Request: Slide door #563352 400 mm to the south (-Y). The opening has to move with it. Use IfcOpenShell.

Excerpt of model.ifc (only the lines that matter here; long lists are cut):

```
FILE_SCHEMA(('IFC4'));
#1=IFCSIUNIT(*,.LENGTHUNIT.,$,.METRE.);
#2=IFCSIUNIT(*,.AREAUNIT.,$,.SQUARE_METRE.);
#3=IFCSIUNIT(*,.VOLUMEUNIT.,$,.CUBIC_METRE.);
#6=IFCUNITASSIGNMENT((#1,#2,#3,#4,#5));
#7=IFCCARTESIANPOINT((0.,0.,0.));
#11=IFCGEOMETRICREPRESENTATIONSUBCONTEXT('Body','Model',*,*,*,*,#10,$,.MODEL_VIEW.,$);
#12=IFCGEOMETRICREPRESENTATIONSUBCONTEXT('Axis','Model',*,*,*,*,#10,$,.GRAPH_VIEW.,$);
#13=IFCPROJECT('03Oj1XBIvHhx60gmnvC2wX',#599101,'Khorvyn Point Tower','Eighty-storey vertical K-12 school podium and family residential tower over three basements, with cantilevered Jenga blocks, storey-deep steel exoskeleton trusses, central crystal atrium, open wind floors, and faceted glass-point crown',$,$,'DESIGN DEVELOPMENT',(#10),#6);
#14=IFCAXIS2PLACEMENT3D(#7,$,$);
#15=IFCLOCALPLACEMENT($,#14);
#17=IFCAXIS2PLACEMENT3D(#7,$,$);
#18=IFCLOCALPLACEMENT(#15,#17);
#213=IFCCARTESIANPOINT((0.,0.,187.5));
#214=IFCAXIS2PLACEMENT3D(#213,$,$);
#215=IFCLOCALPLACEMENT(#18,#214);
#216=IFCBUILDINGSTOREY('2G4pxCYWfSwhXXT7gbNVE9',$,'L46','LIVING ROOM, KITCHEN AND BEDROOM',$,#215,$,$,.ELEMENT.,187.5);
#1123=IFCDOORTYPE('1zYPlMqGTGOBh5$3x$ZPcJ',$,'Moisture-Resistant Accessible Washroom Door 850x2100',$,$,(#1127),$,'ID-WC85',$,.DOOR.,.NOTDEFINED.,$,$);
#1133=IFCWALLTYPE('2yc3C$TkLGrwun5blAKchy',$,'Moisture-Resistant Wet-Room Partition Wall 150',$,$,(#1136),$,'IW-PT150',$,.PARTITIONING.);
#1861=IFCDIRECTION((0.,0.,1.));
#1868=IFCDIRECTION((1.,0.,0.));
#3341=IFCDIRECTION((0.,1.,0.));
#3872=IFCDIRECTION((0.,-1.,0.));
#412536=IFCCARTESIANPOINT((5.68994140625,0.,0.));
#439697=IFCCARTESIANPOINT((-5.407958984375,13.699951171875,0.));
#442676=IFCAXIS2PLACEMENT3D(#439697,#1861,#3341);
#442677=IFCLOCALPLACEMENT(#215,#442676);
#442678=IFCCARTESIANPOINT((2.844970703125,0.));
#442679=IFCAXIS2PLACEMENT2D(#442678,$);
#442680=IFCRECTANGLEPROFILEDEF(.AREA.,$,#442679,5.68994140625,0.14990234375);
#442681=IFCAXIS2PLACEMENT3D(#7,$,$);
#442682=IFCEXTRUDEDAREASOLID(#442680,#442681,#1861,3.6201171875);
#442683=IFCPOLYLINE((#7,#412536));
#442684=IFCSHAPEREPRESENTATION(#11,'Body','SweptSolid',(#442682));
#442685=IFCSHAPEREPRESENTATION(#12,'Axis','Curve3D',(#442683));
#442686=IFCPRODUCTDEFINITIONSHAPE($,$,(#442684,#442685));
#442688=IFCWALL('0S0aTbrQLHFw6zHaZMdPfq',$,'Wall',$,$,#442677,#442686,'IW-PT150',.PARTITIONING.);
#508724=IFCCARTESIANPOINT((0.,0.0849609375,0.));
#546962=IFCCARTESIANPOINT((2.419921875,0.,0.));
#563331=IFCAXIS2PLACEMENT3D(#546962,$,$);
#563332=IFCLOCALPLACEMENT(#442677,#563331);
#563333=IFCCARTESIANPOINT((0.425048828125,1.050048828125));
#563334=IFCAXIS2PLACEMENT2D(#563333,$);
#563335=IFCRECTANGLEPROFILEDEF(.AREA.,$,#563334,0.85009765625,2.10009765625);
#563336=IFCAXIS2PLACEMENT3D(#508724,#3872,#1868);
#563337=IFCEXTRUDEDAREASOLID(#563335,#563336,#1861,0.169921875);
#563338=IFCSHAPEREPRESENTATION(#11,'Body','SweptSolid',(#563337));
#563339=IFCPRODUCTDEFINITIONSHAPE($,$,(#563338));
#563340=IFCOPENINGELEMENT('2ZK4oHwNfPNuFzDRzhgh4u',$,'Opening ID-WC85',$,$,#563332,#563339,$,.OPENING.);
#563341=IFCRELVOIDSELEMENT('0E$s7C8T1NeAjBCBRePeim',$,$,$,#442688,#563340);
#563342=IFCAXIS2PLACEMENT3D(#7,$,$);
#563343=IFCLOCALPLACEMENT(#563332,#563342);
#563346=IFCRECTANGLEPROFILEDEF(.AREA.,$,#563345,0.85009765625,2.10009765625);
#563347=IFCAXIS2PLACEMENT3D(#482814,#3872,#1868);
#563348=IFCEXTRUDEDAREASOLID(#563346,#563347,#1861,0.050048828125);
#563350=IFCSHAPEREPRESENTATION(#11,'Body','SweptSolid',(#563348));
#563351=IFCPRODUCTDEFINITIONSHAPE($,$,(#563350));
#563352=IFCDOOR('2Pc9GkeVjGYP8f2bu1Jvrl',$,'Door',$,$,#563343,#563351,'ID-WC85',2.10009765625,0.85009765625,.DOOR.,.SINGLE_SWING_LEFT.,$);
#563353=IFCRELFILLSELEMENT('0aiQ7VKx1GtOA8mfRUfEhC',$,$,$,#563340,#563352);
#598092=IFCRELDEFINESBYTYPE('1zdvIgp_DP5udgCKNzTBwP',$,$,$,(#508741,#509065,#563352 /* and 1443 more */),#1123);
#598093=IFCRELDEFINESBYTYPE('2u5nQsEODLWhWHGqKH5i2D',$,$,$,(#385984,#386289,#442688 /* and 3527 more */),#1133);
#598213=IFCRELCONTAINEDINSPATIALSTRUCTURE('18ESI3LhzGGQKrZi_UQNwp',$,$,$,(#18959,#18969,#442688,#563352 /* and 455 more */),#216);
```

```python
import ifcopenshell
import ifcopenshell.api.geometry
import ifcopenshell.util.placement

model = ifcopenshell.open("model.ifc")

door = model.by_guid("2Pc9GkeVjGYP8f2bu1Jvrl")
opening = door.FillsVoids[0].RelatingOpeningElement
wall = opening.VoidsElements[0].RelatingBuildingElement

wall_matrix = ifcopenshell.util.placement.get_local_placement(wall.ObjectPlacement)
shift = wall_matrix[:3, 0] * -0.4
before = ifcopenshell.util.placement.get_local_placement(door.ObjectPlacement)[:3, 3].copy()

# The door is placed relative to its opening, so it follows when the opening moves.
matrix = ifcopenshell.util.placement.get_local_placement(opening.ObjectPlacement)
matrix[:3, 3] += shift
ifcopenshell.api.geometry.edit_object_placement(
    model, product=opening, matrix=matrix, is_si=False, should_transform_children=True
)

after = ifcopenshell.util.placement.get_local_placement(door.ObjectPlacement)[:3, 3]
print("door moved by", (after - before).round(3) + 0.0)

model.write("model_edited.ifc")
```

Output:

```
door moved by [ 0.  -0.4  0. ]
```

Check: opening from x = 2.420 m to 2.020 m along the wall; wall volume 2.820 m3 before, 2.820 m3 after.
